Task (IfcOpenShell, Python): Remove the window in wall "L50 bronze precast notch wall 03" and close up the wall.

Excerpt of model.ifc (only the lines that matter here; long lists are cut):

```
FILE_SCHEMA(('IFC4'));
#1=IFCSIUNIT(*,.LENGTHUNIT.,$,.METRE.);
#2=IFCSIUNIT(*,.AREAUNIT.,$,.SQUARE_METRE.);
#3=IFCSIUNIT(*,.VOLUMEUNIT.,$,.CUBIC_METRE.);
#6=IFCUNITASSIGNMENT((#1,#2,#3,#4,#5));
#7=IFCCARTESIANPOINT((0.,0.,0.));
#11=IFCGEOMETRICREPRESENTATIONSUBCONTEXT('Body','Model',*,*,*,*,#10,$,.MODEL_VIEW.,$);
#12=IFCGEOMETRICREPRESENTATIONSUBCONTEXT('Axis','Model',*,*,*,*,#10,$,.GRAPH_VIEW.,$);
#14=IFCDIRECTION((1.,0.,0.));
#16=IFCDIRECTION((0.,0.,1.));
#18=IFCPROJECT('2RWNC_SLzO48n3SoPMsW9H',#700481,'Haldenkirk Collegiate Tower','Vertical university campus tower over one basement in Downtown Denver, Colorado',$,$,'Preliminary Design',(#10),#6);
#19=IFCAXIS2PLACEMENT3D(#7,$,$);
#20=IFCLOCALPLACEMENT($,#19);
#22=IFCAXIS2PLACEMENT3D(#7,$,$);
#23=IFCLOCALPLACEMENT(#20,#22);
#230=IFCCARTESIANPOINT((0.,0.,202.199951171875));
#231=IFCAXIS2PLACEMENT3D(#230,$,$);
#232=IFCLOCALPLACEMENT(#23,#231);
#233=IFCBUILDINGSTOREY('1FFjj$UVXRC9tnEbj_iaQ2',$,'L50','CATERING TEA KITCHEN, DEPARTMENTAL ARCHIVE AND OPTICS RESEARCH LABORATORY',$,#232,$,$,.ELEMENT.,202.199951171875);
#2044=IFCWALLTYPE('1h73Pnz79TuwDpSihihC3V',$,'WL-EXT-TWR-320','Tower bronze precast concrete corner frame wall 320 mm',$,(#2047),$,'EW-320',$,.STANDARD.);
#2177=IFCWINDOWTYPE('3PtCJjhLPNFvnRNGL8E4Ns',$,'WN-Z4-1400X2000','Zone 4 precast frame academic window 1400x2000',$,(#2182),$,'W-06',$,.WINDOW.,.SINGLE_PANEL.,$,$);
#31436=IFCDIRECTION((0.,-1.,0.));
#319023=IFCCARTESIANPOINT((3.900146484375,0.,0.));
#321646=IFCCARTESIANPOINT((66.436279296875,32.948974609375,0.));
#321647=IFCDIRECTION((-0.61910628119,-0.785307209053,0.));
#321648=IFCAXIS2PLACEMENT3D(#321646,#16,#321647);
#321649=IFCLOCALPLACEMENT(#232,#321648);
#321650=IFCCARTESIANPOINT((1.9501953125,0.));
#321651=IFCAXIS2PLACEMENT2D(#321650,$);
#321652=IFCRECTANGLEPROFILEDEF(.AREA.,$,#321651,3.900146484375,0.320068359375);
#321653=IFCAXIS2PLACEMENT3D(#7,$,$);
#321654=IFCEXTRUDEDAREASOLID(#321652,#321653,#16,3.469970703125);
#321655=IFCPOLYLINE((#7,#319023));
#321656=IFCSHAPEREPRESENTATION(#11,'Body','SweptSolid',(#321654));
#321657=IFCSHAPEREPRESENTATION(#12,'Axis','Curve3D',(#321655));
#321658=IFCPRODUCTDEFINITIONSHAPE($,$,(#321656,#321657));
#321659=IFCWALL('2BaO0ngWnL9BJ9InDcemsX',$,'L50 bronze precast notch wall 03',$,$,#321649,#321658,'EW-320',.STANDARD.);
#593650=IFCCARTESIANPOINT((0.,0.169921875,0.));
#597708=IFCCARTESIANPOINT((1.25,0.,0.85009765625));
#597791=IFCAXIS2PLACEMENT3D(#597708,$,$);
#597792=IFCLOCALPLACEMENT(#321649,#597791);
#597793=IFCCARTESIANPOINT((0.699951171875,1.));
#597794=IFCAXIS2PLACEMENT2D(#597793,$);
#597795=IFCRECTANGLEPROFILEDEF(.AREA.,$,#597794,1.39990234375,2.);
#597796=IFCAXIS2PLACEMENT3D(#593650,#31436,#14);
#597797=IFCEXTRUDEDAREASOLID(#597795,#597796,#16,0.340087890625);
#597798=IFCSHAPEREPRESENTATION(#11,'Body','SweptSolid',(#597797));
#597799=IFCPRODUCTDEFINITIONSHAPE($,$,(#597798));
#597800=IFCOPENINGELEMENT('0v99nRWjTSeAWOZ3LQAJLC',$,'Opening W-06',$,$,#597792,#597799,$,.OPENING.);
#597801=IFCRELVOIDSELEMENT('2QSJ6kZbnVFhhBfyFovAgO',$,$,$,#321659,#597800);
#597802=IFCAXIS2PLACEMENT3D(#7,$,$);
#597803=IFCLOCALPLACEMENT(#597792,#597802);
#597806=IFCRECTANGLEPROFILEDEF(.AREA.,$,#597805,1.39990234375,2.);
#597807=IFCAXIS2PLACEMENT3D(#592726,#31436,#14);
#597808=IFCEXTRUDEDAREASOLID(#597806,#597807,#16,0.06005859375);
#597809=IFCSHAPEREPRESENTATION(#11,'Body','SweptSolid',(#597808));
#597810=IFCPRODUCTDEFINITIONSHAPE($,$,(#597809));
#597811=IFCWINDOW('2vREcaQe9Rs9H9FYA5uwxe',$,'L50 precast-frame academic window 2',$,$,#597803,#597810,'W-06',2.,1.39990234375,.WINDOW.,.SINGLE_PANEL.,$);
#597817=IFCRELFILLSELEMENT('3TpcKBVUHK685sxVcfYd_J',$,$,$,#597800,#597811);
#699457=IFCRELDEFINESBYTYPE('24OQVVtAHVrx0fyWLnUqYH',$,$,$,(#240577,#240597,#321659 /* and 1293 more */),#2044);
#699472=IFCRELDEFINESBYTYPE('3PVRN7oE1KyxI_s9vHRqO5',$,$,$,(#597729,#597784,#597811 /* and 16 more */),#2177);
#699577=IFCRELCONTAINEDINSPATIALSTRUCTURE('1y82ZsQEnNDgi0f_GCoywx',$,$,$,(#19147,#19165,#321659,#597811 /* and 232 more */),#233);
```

```python
import ifcopenshell
import ifcopenshell.api.feature
import ifcopenshell.api.root
import ifcopenshell.geom
import ifcopenshell.util.shape

model = ifcopenshell.open("model.ifc")
settings = ifcopenshell.geom.settings()


def volume(element):
    """Net volume in cubic metres, openings subtracted."""
    shape = ifcopenshell.geom.create_shape(settings, element)
    return ifcopenshell.util.shape.get_volume(shape.geometry)


window = model.by_id(597811)
opening = window.FillsVoids[0].RelatingOpeningElement
wall = opening.VoidsElements[0].RelatingBuildingElement
before = volume(wall)

ifcopenshell.api.root.remove_product(model, product=window)
ifcopenshell.api.feature.remove_feature(model, feature=opening)

after = volume(wall)

print(f"wall volume {before:.3f} -> {after:.3f} m3")

model.write("model_rev.ifc")
```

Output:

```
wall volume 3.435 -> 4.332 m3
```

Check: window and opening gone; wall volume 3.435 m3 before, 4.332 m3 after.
